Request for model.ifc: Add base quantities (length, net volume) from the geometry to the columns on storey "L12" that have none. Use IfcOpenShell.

First a look at what the model holds.

```python
import ifcopenshell
import ifcopenshell.util.element
import ifcopenshell.util.unit

model = ifcopenshell.open("model.ifc")
print(model.schema)
for unit_type in ("LENGTHUNIT", "AREAUNIT", "VOLUMEUNIT"):
    print(unit_type, ifcopenshell.util.unit.calculate_unit_scale(model, unit_type))
storey = next(s for s in model.by_type("IfcBuildingStorey") if s.Name == "L12")
columns = [e for e in ifcopenshell.util.element.get_decomposition(storey) if e.is_a("IfcColumn")]
for e in sorted(columns, key=lambda e: e.id()):
    print(e.id(), e.is_a(), e.Name, list(ifcopenshell.util.element.get_psets(e, qtos_only=True)), sep=" | ")
```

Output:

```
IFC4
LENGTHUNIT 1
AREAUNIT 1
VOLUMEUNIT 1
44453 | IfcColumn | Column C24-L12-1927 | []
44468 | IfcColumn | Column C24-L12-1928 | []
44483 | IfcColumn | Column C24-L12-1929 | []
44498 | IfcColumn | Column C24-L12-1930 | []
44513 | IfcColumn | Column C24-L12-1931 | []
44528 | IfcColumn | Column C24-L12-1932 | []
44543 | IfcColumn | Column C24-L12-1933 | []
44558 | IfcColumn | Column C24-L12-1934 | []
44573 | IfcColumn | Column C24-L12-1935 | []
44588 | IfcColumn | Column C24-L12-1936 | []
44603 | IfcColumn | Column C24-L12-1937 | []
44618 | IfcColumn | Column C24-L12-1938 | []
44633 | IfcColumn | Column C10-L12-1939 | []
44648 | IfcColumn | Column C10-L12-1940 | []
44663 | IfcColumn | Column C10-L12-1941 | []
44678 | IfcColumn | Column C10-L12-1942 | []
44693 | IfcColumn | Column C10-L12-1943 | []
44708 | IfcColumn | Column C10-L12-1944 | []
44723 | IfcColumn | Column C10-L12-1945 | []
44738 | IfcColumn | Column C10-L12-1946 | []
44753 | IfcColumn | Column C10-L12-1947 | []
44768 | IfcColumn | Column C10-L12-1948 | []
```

```python
import ifcopenshell
import ifcopenshell.api.pset
import ifcopenshell.geom
import ifcopenshell.util.element
import ifcopenshell.util.shape
import ifcopenshell.util.unit

model = ifcopenshell.open("model.ifc")
unit_scale = ifcopenshell.util.unit.calculate_unit_scale(model)
volume_scale = ifcopenshell.util.unit.calculate_unit_scale(model, "VOLUMEUNIT")
settings = ifcopenshell.geom.settings()

storey = next(s for s in model.by_type("IfcBuildingStorey") if s.Name == "L12")
columns = [e for e in ifcopenshell.util.element.get_decomposition(storey) if e.is_a("IfcColumn")]

for e in sorted(columns, key=lambda e: e.id()):
    if ifcopenshell.util.element.get_psets(e, qtos_only=True, should_inherit=False):
        continue
    # Geometry comes back in metres, in the element's own axes.
    shape = ifcopenshell.geom.create_shape(settings, e)
    values = {
        "Length": ifcopenshell.util.shape.get_z(shape.geometry) / unit_scale,
        "NetVolume": ifcopenshell.util.shape.get_volume(shape.geometry) / volume_scale,
    }
    qto = ifcopenshell.api.pset.add_qto(model, product=e, name="Qto_ColumnBaseQuantities")
    ifcopenshell.api.pset.edit_qto(model, qto=qto, properties=values)
    print(e.id(), {k: round(v, 3) for k, v in values.items()})

model.write("model_edited.ifc")
```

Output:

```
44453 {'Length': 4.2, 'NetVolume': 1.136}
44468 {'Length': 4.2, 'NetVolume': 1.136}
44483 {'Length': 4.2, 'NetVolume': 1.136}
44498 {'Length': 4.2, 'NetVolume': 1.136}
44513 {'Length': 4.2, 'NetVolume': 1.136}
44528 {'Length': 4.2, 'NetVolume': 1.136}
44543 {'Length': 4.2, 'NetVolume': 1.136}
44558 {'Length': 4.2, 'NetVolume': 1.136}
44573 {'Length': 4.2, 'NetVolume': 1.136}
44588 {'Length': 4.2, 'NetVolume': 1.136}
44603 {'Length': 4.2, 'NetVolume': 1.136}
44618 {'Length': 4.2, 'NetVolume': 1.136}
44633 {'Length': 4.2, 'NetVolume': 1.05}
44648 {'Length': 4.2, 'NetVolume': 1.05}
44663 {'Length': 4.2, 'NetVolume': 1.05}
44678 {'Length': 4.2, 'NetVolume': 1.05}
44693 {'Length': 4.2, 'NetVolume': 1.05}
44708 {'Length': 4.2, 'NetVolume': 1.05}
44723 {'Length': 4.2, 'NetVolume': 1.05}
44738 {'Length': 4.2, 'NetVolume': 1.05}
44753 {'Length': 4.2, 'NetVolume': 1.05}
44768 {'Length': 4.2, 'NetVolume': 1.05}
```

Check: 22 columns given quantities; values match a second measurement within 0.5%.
